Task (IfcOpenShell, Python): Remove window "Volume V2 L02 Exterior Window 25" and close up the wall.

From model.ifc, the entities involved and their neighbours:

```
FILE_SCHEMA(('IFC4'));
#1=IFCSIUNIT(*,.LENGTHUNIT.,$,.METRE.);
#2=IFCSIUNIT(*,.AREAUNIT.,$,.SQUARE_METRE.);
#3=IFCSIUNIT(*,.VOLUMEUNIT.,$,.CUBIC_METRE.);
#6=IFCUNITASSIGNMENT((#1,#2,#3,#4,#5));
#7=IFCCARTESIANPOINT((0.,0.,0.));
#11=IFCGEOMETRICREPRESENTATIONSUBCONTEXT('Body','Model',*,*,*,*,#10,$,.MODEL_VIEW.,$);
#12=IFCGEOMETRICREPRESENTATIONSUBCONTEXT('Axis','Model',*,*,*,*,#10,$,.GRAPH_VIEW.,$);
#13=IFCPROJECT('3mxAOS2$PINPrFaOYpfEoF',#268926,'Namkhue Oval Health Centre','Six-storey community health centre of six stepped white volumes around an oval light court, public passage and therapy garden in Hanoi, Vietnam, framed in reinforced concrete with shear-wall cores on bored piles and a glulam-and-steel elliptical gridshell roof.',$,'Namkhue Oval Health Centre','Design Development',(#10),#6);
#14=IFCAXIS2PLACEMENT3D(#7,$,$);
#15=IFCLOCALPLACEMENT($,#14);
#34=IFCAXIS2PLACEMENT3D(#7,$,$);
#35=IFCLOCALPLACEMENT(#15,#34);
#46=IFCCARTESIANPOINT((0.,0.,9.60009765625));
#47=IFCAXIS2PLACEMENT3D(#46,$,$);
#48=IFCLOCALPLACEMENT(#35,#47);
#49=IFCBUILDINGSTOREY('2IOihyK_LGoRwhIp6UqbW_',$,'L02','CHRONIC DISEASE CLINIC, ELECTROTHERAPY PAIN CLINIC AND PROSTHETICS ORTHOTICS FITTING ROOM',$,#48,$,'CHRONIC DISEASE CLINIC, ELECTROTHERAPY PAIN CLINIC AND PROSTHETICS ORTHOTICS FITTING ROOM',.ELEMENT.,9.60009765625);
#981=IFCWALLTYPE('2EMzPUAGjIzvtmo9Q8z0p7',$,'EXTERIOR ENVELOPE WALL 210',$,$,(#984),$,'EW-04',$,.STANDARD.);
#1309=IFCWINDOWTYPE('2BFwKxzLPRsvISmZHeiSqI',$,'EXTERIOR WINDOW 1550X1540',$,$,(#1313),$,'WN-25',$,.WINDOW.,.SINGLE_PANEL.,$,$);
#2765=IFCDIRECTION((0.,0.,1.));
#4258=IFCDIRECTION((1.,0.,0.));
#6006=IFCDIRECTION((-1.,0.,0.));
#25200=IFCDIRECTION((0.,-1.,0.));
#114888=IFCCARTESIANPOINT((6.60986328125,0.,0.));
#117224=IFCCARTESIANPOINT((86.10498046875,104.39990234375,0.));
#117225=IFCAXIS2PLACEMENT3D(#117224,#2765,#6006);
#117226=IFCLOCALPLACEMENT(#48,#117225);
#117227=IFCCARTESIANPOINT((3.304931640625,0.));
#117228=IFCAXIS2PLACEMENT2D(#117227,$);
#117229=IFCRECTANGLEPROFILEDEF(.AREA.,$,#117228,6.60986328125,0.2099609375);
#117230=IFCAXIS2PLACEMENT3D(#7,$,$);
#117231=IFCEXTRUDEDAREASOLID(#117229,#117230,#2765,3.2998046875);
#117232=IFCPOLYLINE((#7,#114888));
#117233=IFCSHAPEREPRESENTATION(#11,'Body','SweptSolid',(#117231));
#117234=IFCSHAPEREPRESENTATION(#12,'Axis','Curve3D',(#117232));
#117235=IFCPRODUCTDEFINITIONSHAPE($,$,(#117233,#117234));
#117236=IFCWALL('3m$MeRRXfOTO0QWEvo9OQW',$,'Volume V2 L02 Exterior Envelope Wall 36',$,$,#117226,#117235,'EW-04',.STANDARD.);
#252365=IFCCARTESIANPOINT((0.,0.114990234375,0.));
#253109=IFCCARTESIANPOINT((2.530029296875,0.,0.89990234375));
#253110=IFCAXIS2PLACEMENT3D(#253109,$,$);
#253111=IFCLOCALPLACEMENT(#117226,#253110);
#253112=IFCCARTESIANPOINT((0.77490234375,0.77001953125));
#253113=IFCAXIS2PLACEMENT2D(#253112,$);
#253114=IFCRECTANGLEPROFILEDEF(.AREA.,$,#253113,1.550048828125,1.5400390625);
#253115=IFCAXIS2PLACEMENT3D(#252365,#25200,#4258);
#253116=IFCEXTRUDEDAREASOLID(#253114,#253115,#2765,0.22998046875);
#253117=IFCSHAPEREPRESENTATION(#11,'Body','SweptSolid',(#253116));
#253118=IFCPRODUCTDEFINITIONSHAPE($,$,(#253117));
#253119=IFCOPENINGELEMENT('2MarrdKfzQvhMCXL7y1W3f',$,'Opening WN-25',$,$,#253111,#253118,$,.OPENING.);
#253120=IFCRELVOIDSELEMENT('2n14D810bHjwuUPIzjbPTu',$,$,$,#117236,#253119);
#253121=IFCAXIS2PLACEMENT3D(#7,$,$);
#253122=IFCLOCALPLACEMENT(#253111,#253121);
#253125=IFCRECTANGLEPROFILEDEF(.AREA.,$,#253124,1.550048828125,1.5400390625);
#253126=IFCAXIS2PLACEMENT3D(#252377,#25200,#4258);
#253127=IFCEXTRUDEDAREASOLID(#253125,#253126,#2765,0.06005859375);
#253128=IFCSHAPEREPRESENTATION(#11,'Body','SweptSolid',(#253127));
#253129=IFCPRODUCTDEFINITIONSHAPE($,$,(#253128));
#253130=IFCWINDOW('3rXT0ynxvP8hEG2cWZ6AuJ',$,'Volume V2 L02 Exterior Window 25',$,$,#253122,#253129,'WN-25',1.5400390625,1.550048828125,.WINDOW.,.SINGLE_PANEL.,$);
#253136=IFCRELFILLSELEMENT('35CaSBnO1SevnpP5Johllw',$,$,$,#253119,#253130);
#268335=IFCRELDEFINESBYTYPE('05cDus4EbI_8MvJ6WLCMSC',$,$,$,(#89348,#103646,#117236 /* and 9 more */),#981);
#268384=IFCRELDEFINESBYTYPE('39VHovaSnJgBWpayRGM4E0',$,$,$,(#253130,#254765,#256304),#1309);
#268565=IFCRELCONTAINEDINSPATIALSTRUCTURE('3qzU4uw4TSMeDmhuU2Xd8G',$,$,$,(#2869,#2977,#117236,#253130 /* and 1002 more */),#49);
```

```python
import ifcopenshell
import ifcopenshell.api.feature
import ifcopenshell.api.root
import ifcopenshell.geom
import ifcopenshell.util.shape

model = ifcopenshell.open("model.ifc")
settings = ifcopenshell.geom.settings()


def volume(element):
    """Net volume in cubic metres, openings subtracted."""
    shape = ifcopenshell.geom.create_shape(settings, element)
    return ifcopenshell.util.shape.get_volume(shape.geometry)


window = model.by_id(253130)
opening = window.FillsVoids[0].RelatingOpeningElement
wall = opening.VoidsElements[0].RelatingBuildingElement
before = volume(wall)

ifcopenshell.api.root.remove_product(model, product=window)
ifcopenshell.api.feature.remove_feature(model, feature=opening)

after = volume(wall)

print(f"wall volume {before:.3f} -> {after:.3f} m3")

model.write("model-out.ifc")
```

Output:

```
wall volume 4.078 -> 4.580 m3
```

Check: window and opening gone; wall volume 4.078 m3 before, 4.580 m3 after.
